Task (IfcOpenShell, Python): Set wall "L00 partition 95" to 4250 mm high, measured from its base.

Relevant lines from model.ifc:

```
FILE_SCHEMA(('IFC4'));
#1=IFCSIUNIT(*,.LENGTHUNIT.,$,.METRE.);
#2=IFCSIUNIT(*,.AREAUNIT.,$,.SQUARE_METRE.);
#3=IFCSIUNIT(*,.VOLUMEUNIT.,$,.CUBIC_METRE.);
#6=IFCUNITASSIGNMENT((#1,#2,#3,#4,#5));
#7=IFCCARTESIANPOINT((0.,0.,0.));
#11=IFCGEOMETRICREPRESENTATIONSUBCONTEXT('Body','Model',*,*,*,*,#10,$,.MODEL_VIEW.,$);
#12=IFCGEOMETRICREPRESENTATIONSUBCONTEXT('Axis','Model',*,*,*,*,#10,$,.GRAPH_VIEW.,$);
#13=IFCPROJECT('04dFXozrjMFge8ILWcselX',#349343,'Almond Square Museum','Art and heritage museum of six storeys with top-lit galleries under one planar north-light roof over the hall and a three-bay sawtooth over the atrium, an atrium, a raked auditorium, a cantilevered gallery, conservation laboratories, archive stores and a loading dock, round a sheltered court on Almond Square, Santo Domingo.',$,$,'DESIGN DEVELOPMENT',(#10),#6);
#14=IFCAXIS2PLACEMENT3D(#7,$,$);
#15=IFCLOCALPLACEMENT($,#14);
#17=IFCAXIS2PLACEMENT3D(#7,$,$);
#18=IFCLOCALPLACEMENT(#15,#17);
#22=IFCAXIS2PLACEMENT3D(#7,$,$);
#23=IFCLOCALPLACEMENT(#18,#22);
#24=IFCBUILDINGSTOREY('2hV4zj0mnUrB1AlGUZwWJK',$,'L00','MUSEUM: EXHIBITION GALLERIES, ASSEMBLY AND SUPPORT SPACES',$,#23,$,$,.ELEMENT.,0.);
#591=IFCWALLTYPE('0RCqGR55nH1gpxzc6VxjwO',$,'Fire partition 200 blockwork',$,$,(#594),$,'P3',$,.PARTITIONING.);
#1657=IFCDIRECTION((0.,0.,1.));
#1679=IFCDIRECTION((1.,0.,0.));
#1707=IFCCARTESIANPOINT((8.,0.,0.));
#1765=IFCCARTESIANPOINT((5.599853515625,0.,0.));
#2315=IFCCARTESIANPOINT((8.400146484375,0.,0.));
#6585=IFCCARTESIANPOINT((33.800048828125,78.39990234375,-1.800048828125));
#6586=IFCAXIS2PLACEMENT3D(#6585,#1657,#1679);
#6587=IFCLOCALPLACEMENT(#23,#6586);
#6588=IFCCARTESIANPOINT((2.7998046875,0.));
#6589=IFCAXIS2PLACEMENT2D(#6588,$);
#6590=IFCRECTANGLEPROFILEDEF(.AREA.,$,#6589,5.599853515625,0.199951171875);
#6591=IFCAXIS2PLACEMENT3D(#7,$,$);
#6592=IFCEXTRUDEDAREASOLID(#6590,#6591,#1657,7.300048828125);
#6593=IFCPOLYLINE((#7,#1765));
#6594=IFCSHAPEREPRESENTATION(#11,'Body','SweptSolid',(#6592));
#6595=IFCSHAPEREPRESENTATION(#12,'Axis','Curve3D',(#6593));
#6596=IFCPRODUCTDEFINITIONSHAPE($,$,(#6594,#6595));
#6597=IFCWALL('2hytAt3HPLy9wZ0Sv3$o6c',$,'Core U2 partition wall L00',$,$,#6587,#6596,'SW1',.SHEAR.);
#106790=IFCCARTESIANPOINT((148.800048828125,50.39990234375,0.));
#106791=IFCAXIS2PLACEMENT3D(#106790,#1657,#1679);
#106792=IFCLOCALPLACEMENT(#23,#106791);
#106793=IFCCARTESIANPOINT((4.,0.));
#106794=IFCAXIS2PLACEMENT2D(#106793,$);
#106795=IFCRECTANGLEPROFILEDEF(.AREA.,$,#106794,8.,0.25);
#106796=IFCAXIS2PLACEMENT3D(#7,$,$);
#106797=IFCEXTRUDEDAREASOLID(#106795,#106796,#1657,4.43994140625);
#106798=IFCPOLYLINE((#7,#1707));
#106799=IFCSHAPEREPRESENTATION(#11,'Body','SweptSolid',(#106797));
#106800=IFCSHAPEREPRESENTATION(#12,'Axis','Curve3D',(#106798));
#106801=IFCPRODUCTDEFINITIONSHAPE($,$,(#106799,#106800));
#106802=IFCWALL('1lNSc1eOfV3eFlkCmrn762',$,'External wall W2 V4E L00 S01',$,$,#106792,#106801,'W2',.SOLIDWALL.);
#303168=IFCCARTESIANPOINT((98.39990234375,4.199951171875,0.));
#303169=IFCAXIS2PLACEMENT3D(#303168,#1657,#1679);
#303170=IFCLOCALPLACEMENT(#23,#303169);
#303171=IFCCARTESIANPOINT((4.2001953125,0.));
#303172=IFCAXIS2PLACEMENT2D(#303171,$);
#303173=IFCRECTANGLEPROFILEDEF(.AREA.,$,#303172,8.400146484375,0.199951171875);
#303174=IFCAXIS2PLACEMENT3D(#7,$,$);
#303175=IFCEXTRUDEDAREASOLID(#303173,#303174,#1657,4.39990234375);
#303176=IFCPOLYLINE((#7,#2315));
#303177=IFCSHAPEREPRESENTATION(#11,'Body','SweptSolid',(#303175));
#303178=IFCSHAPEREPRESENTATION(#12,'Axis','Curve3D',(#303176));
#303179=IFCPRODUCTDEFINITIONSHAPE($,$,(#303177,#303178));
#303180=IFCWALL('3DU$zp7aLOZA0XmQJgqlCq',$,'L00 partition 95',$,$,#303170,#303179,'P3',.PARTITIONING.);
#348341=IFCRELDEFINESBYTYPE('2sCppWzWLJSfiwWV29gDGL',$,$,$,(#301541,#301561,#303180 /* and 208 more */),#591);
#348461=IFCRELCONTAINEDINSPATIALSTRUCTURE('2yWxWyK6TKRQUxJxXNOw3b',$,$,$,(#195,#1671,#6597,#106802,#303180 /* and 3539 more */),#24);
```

```python
import ifcopenshell
import ifcopenshell.geom
import ifcopenshell.util.representation
import ifcopenshell.util.shape
import ifcopenshell.util.unit

model = ifcopenshell.open("model.ifc")
unit_scale = ifcopenshell.util.unit.calculate_unit_scale(model)
settings = ifcopenshell.geom.settings()


def volume(element):
    """Net volume in cubic metres, openings subtracted."""
    shape = ifcopenshell.geom.create_shape(settings, element)
    return ifcopenshell.util.shape.get_volume(shape.geometry)


wall = model.by_id(303180)
before = volume(wall)

body = ifcopenshell.util.representation.get_representation(wall, "Model", "Body")
solid = body.Items[0]
old_height = solid.Depth
solid.Depth = 4.25 / unit_scale
after = volume(wall)

print(f"height {old_height:g} -> {solid.Depth:g}, volume {before:.3f} -> {after:.3f} m3")

model.write("model_rev.ifc")
```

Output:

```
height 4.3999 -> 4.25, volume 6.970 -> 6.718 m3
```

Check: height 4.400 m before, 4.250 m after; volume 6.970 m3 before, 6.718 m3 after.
